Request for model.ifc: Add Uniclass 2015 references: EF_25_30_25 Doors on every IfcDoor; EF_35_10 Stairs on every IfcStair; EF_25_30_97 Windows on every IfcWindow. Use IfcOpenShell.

First a look at what the model holds.

```python
import ifcopenshell

model = ifcopenshell.open("model.ifc")
print(model.schema)
print("classifications:", [c.Name for c in model.by_type("IfcClassification")])
for ifc_class in ("IfcDoor", "IfcRoof", "IfcStair", "IfcWall", "IfcWindow"):
    print(ifc_class, len(model.by_type(ifc_class)))
```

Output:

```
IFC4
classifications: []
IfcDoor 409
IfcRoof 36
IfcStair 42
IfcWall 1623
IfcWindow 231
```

```python
import ifcopenshell
import ifcopenshell.api.classification

model = ifcopenshell.open("model.ifc")

system = ifcopenshell.api.classification.add_classification(model, classification="Uniclass 2015")

codes = {
    "IfcDoor": ("EF_25_30_25", "Doors"),
    "IfcStair": ("EF_35_10", "Stairs"),
    "IfcWindow": ("EF_25_30_97", "Windows"),
}
for ifc_class, (code, name) in codes.items():
    products = model.by_type(ifc_class)
    ifcopenshell.api.classification.add_reference(
        model, products=products, classification=system, identification=code, name=name
    )
    print(code, len(products))

model.write("model-out.ifc")
```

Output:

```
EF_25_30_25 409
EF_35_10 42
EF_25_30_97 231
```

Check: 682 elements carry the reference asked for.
